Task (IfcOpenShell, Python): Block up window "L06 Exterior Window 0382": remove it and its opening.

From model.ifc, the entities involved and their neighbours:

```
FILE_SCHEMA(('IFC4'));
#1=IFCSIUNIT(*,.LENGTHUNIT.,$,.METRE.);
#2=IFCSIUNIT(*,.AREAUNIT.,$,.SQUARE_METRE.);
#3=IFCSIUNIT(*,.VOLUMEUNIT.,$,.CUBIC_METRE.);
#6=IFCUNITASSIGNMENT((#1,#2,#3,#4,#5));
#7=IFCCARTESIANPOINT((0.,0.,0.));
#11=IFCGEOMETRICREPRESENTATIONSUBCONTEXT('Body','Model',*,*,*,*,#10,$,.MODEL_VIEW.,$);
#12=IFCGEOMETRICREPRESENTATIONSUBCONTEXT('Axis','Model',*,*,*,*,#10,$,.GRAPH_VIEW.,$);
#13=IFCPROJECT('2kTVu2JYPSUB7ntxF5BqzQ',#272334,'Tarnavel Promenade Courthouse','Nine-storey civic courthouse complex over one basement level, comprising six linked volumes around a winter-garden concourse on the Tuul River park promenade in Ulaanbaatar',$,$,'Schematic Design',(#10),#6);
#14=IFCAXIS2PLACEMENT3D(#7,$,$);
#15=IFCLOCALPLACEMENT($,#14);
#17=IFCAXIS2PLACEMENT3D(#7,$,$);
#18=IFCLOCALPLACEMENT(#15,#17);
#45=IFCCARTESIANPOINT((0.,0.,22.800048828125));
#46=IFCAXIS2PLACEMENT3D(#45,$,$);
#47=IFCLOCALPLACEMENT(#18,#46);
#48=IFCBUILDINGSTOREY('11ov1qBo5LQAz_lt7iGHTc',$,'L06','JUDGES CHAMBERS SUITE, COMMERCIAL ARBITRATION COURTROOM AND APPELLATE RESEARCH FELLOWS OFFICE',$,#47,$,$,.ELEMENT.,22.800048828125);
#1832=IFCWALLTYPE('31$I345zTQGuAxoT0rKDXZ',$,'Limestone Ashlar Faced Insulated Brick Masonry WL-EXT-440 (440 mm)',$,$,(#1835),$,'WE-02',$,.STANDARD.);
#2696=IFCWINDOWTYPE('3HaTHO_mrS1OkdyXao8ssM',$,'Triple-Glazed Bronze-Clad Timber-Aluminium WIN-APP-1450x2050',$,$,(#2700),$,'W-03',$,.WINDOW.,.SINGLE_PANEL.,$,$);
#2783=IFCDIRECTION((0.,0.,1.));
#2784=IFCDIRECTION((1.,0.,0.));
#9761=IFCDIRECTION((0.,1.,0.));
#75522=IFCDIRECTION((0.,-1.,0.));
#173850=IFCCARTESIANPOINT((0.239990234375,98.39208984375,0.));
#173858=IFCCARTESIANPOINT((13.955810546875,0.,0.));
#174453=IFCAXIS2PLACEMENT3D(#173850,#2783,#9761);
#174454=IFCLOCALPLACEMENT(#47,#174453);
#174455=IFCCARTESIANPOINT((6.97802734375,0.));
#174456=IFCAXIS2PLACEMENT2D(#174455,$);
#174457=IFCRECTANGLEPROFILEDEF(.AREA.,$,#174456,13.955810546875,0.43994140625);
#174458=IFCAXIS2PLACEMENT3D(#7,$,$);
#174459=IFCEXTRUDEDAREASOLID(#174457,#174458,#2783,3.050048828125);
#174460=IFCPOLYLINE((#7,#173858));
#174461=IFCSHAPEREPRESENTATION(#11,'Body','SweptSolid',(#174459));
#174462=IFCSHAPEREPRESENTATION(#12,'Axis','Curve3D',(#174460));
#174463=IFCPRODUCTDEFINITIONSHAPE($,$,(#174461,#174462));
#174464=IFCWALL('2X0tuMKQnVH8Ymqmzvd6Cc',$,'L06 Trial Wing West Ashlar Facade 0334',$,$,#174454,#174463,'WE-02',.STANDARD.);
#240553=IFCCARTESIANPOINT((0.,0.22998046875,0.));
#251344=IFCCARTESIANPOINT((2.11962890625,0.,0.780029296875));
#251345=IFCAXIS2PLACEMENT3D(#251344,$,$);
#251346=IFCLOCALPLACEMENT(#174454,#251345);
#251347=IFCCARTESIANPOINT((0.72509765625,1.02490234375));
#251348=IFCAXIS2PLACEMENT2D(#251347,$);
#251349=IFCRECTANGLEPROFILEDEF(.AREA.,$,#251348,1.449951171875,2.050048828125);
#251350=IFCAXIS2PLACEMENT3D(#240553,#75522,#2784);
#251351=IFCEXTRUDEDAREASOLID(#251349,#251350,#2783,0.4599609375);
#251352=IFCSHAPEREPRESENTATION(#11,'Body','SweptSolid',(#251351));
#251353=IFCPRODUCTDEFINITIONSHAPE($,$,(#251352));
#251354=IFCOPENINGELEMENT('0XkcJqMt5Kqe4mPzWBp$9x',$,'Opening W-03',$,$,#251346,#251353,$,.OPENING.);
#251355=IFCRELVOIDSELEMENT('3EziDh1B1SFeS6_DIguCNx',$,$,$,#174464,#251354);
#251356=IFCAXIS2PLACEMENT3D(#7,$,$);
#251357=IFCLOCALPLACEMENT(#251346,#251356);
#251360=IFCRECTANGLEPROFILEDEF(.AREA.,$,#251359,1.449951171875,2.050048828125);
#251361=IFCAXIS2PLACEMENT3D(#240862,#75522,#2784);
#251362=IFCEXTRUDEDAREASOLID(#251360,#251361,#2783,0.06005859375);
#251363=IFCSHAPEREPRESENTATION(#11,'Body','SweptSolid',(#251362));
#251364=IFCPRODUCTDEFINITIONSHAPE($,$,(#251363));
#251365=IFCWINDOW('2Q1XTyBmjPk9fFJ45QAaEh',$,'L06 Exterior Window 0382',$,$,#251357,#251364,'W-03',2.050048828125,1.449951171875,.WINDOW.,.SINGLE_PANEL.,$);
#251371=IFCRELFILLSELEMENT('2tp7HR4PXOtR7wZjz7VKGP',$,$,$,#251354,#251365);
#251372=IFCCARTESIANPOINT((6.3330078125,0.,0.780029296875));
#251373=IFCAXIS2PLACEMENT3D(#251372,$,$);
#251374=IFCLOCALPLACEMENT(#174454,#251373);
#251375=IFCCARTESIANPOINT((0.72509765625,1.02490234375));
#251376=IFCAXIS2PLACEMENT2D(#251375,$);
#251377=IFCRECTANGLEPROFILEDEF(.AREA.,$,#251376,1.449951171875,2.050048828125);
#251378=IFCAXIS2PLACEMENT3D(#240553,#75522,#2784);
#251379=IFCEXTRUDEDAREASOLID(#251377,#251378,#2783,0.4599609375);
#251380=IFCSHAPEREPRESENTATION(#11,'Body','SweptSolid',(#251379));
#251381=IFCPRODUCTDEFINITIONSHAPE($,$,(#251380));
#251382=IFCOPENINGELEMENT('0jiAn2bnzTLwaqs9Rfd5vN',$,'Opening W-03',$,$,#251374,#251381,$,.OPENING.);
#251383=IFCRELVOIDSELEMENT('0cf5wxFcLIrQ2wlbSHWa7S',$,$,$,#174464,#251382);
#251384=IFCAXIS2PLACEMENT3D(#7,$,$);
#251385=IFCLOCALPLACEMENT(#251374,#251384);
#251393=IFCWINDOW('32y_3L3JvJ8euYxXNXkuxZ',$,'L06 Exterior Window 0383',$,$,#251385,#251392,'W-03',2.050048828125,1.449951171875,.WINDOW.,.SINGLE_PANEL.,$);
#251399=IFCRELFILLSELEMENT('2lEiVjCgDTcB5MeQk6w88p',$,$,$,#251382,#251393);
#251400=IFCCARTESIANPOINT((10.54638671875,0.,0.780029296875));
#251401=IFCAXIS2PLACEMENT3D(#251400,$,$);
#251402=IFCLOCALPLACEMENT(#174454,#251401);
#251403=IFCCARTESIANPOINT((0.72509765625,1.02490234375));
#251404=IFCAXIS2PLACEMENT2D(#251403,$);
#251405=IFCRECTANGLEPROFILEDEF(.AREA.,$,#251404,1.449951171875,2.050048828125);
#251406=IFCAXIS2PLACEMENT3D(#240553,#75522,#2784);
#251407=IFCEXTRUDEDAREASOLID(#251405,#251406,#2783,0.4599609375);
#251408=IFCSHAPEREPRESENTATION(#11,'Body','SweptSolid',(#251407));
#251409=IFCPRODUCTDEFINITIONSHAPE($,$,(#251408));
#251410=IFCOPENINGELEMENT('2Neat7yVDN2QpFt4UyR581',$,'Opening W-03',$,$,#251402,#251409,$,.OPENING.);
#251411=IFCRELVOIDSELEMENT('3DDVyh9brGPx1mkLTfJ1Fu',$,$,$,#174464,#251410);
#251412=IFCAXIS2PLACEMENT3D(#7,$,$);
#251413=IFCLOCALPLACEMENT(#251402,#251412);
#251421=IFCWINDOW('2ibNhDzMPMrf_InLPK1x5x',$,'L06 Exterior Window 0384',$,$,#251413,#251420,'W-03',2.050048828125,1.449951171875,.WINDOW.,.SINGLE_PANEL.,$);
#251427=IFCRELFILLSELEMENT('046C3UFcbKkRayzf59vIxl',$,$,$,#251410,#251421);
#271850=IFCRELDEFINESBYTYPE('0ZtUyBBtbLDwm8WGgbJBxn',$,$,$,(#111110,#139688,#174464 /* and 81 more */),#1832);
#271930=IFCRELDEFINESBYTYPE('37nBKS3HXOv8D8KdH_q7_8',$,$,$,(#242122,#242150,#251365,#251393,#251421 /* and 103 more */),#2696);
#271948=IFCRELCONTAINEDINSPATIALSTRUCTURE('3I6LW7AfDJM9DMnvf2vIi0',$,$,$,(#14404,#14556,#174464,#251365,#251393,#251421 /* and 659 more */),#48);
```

```python
import ifcopenshell
import ifcopenshell.api.feature
import ifcopenshell.api.root
import ifcopenshell.geom
import ifcopenshell.util.shape

model = ifcopenshell.open("model.ifc")
settings = ifcopenshell.geom.settings()


def volume(element):
    """Net volume in cubic metres, openings subtracted."""
    shape = ifcopenshell.geom.create_shape(settings, element)
    return ifcopenshell.util.shape.get_volume(shape.geometry)


window = model.by_guid("2Q1XTyBmjPk9fFJ45QAaEh")
opening = window.FillsVoids[0].RelatingOpeningElement
wall = opening.VoidsElements[0].RelatingBuildingElement
before = volume(wall)

ifcopenshell.api.root.remove_product(model, product=window)
ifcopenshell.api.feature.remove_feature(model, feature=opening)

after = volume(wall)

print(f"wall volume {before:.3f} -> {after:.3f} m3")

model.write("model_edited.ifc")
```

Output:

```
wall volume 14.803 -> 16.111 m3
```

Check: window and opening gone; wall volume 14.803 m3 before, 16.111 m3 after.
